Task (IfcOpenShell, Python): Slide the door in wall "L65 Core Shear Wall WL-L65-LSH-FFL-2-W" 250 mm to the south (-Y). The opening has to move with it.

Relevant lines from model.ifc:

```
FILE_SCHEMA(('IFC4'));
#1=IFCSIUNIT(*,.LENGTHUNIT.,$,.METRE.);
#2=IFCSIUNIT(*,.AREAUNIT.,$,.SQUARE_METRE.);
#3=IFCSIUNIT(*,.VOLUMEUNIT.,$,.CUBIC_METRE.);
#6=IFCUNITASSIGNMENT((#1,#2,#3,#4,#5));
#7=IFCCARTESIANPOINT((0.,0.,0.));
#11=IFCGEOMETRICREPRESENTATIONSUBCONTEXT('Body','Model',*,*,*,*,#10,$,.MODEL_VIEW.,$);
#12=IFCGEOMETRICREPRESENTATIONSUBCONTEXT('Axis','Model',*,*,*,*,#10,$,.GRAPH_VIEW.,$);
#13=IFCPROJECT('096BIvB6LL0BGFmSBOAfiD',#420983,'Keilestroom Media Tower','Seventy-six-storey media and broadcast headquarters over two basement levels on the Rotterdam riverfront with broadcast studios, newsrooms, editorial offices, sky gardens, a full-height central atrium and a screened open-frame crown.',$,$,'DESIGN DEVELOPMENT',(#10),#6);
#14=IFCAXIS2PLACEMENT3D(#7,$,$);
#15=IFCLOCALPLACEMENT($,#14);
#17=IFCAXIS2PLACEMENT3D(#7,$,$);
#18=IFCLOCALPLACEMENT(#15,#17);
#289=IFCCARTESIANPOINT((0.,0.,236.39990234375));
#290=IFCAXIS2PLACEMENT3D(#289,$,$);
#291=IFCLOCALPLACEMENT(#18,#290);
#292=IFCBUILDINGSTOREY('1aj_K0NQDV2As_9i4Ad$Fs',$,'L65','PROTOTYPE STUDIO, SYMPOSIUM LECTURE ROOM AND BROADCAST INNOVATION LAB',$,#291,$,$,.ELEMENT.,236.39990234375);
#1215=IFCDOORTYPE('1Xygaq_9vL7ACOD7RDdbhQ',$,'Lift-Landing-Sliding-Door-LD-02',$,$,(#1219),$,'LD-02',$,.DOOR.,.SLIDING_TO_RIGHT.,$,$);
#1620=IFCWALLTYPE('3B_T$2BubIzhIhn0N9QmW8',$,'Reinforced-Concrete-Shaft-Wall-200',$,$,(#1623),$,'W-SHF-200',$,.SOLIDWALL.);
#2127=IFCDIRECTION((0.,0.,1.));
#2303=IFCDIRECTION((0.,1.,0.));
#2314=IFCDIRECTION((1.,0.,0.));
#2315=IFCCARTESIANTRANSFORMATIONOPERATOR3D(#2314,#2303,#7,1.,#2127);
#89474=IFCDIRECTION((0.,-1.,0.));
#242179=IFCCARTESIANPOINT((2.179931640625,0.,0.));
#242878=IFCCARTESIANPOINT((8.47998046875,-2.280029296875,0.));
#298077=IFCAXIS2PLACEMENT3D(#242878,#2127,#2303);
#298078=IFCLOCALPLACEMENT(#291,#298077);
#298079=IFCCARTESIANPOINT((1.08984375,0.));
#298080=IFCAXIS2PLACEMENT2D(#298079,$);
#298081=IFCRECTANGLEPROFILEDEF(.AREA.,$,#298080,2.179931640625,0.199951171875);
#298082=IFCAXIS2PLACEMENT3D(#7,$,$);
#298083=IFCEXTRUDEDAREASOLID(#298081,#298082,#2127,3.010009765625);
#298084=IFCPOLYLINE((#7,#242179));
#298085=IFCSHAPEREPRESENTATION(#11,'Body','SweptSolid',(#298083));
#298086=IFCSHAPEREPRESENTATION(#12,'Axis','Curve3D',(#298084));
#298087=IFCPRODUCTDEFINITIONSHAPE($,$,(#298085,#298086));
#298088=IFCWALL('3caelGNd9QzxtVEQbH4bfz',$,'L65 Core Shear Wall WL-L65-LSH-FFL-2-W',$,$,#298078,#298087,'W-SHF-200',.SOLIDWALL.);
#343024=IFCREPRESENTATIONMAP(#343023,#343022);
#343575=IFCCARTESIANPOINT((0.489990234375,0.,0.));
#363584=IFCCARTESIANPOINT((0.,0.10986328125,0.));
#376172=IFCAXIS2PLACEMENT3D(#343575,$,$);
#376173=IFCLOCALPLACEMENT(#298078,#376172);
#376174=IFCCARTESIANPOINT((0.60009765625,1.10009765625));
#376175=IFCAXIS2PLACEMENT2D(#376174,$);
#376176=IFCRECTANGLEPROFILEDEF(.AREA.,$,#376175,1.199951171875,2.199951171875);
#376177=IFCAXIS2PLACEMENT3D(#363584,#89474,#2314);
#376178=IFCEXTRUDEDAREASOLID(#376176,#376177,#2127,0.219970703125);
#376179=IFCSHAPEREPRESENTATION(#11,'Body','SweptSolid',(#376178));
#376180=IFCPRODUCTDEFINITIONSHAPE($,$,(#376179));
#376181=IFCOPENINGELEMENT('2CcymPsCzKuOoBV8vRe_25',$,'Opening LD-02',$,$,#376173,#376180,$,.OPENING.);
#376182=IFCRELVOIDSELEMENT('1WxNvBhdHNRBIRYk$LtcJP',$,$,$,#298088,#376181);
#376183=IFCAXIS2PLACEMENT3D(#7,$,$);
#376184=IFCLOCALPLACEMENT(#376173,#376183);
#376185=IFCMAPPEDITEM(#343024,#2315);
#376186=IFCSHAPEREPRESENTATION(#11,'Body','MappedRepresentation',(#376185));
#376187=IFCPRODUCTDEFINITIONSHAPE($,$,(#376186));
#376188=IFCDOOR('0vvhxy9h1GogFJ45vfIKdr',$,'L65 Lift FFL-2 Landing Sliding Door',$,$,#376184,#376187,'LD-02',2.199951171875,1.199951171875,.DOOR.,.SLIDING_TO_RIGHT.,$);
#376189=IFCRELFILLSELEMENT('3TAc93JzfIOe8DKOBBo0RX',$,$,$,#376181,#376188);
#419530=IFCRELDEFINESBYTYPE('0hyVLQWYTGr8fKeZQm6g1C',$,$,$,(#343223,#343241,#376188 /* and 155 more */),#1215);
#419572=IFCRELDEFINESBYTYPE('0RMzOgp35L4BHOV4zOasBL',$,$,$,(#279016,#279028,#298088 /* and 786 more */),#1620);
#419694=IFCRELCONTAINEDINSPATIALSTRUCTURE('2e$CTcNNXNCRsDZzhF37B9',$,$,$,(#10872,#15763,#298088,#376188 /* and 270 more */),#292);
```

```python
import ifcopenshell
import ifcopenshell.api.geometry
import ifcopenshell.util.placement
import ifcopenshell.util.unit

model = ifcopenshell.open("model.ifc")
unit_scale = ifcopenshell.util.unit.calculate_unit_scale(model)

door = model.by_guid("0vvhxy9h1GogFJ45vfIKdr")
opening = door.FillsVoids[0].RelatingOpeningElement
wall = opening.VoidsElements[0].RelatingBuildingElement

wall_matrix = ifcopenshell.util.placement.get_local_placement(wall.ObjectPlacement)
shift = wall_matrix[:3, 0] * -0.25 / unit_scale
before = ifcopenshell.util.placement.get_local_placement(door.ObjectPlacement)[:3, 3].copy()

# The door is placed relative to its opening, so it follows when the opening moves.
matrix = ifcopenshell.util.placement.get_local_placement(opening.ObjectPlacement)
matrix[:3, 3] += shift
ifcopenshell.api.geometry.edit_object_placement(
    model, product=opening, matrix=matrix, is_si=False, should_transform_children=True
)

after = ifcopenshell.util.placement.get_local_placement(door.ObjectPlacement)[:3, 3]
print("door moved by", (after - before).round(3) + 0.0)

model.write("model-out.ifc")
```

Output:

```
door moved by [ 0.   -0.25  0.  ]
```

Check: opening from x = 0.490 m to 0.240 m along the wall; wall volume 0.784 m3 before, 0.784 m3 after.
